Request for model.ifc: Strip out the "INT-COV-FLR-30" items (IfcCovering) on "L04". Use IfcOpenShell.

First a look at what the model holds.

```python
import ifcopenshell
import ifcopenshell.util.element

model = ifcopenshell.open("model.ifc")
print(model.schema)
storey = next(s for s in model.by_type("IfcBuildingStorey") if s.Name == "L04")
coverings = [e for e in ifcopenshell.util.element.get_decomposition(storey) if e.is_a("IfcCovering")]
seen = {}
for e in coverings:
    element_type = ifcopenshell.util.element.get_type(e)
    name = element_type.Name if element_type not in (None, e) else None
    seen[name] = seen.get(name, 0) + 1
for name, count in sorted(seen.items(), key=str):
    print(count, "x", name)
```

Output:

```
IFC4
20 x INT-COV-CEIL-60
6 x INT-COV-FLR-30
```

```python
import ifcopenshell
import ifcopenshell.api.root
import ifcopenshell.util.element

model = ifcopenshell.open("model.ifc")

storey = next(s for s in model.by_type("IfcBuildingStorey") if s.Name == "L04")
coverings = [e for e in ifcopenshell.util.element.get_decomposition(storey) if e.is_a("IfcCovering")]
targets = [e for e in coverings if (t := ifcopenshell.util.element.get_type(e)) not in (None, e) and t.Name == "INT-COV-FLR-30"]

for e in targets:
    ifcopenshell.api.root.remove_product(model, product=e)
print(len(targets), "removed")

model.write("model_v2.ifc")
```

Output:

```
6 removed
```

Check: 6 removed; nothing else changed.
